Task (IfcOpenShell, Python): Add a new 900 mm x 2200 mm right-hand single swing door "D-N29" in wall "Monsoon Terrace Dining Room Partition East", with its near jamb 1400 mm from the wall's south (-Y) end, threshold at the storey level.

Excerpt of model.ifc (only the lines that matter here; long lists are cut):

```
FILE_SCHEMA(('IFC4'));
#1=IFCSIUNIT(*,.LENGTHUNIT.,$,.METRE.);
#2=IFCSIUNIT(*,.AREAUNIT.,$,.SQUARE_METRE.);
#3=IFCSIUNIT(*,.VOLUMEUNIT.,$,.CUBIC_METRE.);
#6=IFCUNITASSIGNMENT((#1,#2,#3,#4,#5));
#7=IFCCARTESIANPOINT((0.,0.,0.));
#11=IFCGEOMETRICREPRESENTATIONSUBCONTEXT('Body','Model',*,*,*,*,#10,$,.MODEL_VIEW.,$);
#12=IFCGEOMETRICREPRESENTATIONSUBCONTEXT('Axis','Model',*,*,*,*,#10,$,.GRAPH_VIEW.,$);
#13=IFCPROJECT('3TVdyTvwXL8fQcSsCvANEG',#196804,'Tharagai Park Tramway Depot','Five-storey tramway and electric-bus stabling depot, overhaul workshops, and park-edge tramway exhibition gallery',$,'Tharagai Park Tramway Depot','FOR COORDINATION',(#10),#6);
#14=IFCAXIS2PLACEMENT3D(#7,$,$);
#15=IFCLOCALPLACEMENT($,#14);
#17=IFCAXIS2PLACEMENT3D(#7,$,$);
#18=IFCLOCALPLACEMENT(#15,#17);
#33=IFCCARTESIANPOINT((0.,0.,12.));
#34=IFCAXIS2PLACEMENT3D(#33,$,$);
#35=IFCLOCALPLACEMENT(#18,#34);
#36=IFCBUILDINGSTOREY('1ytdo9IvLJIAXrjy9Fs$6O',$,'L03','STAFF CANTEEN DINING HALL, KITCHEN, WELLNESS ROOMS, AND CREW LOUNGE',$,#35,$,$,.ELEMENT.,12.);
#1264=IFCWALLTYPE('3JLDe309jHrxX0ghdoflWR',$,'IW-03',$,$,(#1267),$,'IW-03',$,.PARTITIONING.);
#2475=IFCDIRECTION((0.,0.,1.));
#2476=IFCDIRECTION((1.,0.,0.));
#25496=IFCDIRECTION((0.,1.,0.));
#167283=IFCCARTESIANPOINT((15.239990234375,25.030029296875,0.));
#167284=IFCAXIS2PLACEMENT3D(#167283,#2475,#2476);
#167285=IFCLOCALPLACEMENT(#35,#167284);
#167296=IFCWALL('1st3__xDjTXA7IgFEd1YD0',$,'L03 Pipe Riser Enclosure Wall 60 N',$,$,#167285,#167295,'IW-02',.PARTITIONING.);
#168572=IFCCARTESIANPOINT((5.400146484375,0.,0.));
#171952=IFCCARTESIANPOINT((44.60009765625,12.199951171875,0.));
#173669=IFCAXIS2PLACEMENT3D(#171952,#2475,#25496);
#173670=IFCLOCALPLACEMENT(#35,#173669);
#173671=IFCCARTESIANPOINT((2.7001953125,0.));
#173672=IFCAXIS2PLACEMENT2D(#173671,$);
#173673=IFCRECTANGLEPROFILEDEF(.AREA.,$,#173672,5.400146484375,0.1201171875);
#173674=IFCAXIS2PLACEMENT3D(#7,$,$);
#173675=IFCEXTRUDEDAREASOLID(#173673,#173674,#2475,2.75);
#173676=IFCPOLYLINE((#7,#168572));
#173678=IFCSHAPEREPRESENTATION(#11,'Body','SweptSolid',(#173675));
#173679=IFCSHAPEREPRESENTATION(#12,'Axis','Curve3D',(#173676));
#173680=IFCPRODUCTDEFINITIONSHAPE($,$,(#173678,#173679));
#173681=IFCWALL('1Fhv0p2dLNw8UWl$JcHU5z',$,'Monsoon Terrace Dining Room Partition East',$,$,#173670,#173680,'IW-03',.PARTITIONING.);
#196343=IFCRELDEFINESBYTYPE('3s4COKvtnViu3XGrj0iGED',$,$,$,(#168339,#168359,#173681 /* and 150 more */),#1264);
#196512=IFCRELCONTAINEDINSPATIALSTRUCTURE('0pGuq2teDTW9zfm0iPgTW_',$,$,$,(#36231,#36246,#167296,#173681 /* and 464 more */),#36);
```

```python
import numpy as np
import ifcopenshell
import ifcopenshell.api.feature
import ifcopenshell.api.geometry
import ifcopenshell.api.root
import ifcopenshell.api.spatial
import ifcopenshell.geom
import ifcopenshell.util.element
import ifcopenshell.util.placement
import ifcopenshell.util.representation
import ifcopenshell.util.shape
import ifcopenshell.util.unit

model = ifcopenshell.open("model.ifc")
unit_scale = ifcopenshell.util.unit.calculate_unit_scale(model)
settings = ifcopenshell.geom.settings()


def volume(element):
    """Net volume in cubic metres, openings subtracted."""
    shape = ifcopenshell.geom.create_shape(settings, element)
    return ifcopenshell.util.shape.get_volume(shape.geometry)


wall = model.by_guid("1Fhv0p2dLNw8UWl$JcHU5z")
storey = ifcopenshell.util.element.get_container(wall, ifc_class="IfcBuildingStorey")
context = ifcopenshell.util.representation.get_context(model, "Model", "Body", "MODEL_VIEW")
before = volume(wall)

width, height, from_end, sill = 0.9, 2.2, 1.4, 0.0  # metres

# The wall runs along its own X axis, and the end named is its -X end.
wall_shape = ifcopenshell.geom.create_shape(settings, wall)
x, y, z = ifcopenshell.util.shape.get_vertices(wall_shape.geometry).T
start = x.min() + from_end
face, thickness = float(y.min()), float(y.max() - y.min())
wall_matrix = ifcopenshell.util.placement.get_local_placement(wall.ObjectPlacement)
level = ifcopenshell.util.placement.get_local_placement(storey.ObjectPlacement)[2, 3]


def in_wall(x, y):
    """Placement at x, y metres in the wall's axes, at sill height."""
    matrix = wall_matrix.copy()
    matrix[:, 3] = wall_matrix @ np.array([x / unit_scale, y / unit_scale, 0.0, 1.0])
    matrix[2, 3] = level + sill / unit_scale
    return matrix


# Opening: a box that overshoots both wall faces by 50 mm.
opening = ifcopenshell.api.root.create_entity(model, ifc_class="IfcOpeningElement", predefined_type="OPENING")
box = ifcopenshell.api.geometry.add_wall_representation(
    model, context=context, length=width, height=height, thickness=thickness + 0.1
)
ifcopenshell.api.geometry.assign_representation(model, product=opening, representation=box)
ifcopenshell.api.geometry.edit_object_placement(model, product=opening, matrix=in_wall(start, face - 0.05), is_si=False)
ifcopenshell.api.feature.add_feature(model, feature=opening, element=wall)

door = ifcopenshell.api.root.create_entity(model, ifc_class="IfcDoor", name="D-N29", predefined_type="DOOR")
door.OverallWidth, door.OverallHeight = width / unit_scale, height / unit_scale
door.OperationType = "SINGLE_SWING_RIGHT"
body = ifcopenshell.api.geometry.add_door_representation(
    model,
    context=context,
    overall_width=door.OverallWidth,
    overall_height=door.OverallHeight,
    operation_type="SINGLE_SWING_RIGHT",
    lining_properties={"LiningDepth": thickness / unit_scale, "ThresholdDepth": thickness / unit_scale},
)
ifcopenshell.api.geometry.assign_representation(model, product=door, representation=body)
ifcopenshell.api.spatial.assign_container(model, products=[door], relating_structure=storey)
ifcopenshell.api.feature.add_filling(model, opening=opening, element=door)

# The lining spans the wall, so the door starts at the wall face.
ifcopenshell.api.geometry.edit_object_placement(model, product=door, matrix=in_wall(start, face), is_si=False)

after = volume(wall)

print(f"wall volume {before:.3f} -> {after:.3f} m3")

model.write("model-out.ifc")
```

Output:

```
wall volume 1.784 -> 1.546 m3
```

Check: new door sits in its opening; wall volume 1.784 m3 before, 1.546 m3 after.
